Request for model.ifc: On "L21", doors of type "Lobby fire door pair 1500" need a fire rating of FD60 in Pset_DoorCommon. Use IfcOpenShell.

First a look at what the model holds.

```python
import ifcopenshell
import ifcopenshell.util.element

model = ifcopenshell.open("model.ifc")
print(model.schema)
storey = next(s for s in model.by_type("IfcBuildingStorey") if s.Name == "L21")
doors = [e for e in ifcopenshell.util.element.get_decomposition(storey) if e.is_a("IfcDoor")]
seen = {}
for e in doors:
    element_type = ifcopenshell.util.element.get_type(e)
    key = (element_type.Name if element_type != e and element_type else None, ifcopenshell.util.element.get_pset(e, "Pset_DoorCommon", "FireRating"))
    seen[key] = seen.get(key, 0) + 1
for (name, value), count in sorted(seen.items(), key=str):
    print(count, "x", name, "|", value)
```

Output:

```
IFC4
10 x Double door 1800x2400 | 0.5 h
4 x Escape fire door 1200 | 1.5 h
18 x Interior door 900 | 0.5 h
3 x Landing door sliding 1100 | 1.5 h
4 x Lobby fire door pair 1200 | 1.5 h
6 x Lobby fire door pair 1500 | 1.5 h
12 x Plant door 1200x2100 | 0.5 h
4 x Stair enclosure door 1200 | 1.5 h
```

```python
import ifcopenshell
import ifcopenshell.api.pset
import ifcopenshell.util.element

model = ifcopenshell.open("model.ifc")

storey = next(s for s in model.by_type("IfcBuildingStorey") if s.Name == "L21")
doors = [e for e in ifcopenshell.util.element.get_decomposition(storey) if e.is_a("IfcDoor")]

count = 0
for e in doors:
    element_type = ifcopenshell.util.element.get_type(e)
    if element_type in (None, e) or element_type.Name != "Lobby fire door pair 1500":
        continue
    found = ifcopenshell.util.element.get_pset(e, "Pset_DoorCommon", should_inherit=False)
    if found:
        pset = model.by_id(found["id"])
        if len(ifcopenshell.util.element.get_elements_by_pset(pset)) > 1:
            pset = ifcopenshell.api.pset.unshare_pset(model, products=[e], pset=pset)[0]
    else:
        pset = ifcopenshell.api.pset.add_pset(model, product=e, name="Pset_DoorCommon")
    ifcopenshell.api.pset.edit_pset(model, pset=pset, properties={"FireRating": "FD60"})
    count += 1

print(count, "doors updated")

model.write("model-out.ifc")
```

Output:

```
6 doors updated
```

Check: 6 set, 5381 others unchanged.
